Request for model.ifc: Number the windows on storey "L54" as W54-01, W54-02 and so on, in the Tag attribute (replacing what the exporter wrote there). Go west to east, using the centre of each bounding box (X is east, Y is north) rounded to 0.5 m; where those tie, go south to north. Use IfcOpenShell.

First a look at what the model holds.

```python
import ifcopenshell
import ifcopenshell.util.element
import ifcopenshell.util.placement

model = ifcopenshell.open("model.ifc")
print(model.schema)
storey = next(s for s in model.by_type("IfcBuildingStorey") if s.Name == "L54")
windows = [e for e in ifcopenshell.util.element.get_decomposition(storey) if e.is_a("IfcWindow")]
for e in sorted(windows, key=lambda e: e.id()):
    origin = ifcopenshell.util.placement.get_local_placement(e.ObjectPlacement)[:3, 3]
    print(e.id(), e.Tag, e.Name, origin.round(2) + 0.0, sep=" | ")
```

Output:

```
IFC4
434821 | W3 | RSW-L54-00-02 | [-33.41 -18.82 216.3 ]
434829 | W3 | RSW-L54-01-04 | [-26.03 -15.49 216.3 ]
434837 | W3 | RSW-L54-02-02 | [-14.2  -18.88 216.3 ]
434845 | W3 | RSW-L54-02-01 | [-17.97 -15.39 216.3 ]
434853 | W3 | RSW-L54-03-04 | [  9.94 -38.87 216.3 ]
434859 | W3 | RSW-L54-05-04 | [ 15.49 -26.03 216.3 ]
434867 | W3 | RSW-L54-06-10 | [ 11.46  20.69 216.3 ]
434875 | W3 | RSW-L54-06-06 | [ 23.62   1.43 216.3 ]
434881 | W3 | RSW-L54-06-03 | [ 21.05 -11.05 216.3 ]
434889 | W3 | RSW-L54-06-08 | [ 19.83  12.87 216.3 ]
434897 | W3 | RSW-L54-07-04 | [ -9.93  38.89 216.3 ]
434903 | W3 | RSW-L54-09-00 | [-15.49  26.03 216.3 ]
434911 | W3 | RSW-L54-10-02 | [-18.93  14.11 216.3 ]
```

```python
import ifcopenshell
import ifcopenshell.geom
import ifcopenshell.util.element
import ifcopenshell.util.shape

model = ifcopenshell.open("model.ifc")
settings = ifcopenshell.geom.settings()
settings.set("use-world-coords", True)


def centre(element):
    shape = ifcopenshell.geom.create_shape(settings, element)
    return ifcopenshell.util.shape.get_bbox_centroid(shape.geometry)


storey = next(s for s in model.by_type("IfcBuildingStorey") if s.Name == "L54")
windows = [e for e in ifcopenshell.util.element.get_decomposition(storey) if e.is_a("IfcWindow")]

# Insertion points can sit at a corner or the storey origin, so sort by the geometry (in metres).
centres = {e: centre(e) for e in windows}
windows.sort(key=lambda e: (round(centres[e][0] / 0.5), centres[e][1]))

for i, e in enumerate(windows, start=1):
    number = f"W54-{i:02d}"
    e.Tag = number
    print(e.id(), number)

model.write("model_updated.ifc")
```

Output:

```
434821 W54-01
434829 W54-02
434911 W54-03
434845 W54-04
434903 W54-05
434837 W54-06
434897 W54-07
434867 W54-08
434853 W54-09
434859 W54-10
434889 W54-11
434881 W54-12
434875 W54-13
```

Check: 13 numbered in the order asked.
